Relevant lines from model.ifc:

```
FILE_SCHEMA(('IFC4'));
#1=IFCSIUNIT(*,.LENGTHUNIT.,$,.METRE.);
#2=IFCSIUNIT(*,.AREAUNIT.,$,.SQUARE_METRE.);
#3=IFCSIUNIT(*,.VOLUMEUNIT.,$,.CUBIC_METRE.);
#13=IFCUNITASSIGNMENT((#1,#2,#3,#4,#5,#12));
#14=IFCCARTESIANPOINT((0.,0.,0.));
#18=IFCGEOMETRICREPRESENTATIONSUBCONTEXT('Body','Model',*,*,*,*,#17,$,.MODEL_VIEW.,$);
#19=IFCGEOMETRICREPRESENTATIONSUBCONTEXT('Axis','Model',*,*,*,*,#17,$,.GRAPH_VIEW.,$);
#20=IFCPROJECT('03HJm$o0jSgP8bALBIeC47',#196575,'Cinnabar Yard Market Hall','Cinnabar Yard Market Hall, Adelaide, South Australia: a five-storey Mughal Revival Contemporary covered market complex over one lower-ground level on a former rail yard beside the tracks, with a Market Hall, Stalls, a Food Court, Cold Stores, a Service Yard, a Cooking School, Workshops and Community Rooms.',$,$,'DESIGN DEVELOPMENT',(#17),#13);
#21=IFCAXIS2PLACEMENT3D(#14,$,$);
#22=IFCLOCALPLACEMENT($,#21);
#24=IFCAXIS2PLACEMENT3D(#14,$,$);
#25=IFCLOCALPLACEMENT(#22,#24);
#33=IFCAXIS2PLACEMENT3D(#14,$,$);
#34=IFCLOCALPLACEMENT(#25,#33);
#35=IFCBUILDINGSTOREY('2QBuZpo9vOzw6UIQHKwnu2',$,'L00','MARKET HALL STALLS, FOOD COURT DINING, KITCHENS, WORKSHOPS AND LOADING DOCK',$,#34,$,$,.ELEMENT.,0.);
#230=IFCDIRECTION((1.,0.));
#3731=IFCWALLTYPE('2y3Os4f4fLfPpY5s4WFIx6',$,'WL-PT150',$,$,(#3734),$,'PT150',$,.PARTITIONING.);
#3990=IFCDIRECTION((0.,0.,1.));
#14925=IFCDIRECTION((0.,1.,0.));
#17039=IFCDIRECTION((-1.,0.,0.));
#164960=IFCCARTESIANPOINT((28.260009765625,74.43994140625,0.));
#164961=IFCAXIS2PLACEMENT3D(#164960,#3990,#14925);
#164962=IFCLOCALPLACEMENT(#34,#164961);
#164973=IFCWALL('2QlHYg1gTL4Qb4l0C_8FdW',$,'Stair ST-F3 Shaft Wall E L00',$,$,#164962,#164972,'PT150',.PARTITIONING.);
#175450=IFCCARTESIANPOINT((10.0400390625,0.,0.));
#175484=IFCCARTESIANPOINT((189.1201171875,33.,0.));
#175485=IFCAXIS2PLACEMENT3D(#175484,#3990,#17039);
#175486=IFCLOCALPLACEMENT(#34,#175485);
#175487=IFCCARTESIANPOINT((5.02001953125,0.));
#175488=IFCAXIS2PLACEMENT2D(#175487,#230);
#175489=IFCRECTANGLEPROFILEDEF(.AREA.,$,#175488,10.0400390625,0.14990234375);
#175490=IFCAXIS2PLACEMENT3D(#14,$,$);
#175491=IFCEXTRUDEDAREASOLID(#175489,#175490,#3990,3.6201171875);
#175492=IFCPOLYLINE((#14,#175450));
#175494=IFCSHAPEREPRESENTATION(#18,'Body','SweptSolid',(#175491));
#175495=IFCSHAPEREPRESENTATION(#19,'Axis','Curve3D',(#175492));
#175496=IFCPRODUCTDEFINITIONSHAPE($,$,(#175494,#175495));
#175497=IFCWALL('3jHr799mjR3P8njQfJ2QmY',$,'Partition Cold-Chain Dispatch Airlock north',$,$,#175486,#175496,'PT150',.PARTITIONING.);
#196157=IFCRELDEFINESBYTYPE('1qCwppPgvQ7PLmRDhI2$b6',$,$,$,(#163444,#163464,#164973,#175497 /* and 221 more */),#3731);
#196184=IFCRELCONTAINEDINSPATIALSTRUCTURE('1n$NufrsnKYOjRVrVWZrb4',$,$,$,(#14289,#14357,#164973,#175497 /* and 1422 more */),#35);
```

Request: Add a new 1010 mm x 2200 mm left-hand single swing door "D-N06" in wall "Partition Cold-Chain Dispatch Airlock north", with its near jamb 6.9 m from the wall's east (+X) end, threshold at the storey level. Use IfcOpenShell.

```python
import numpy as np
import ifcopenshell
import ifcopenshell.api.feature
import ifcopenshell.api.geometry
import ifcopenshell.api.root
import ifcopenshell.api.spatial
import ifcopenshell.geom
import ifcopenshell.util.element
import ifcopenshell.util.placement
import ifcopenshell.util.representation
import ifcopenshell.util.shape
import ifcopenshell.util.unit

model = ifcopenshell.open("model.ifc")
unit_scale = ifcopenshell.util.unit.calculate_unit_scale(model)
settings = ifcopenshell.geom.settings()


def volume(element):
    """Net volume in cubic metres, openings subtracted."""
    shape = ifcopenshell.geom.create_shape(settings, element)
    return ifcopenshell.util.shape.get_volume(shape.geometry)


wall = model.by_guid("3jHr799mjR3P8njQfJ2QmY")
storey = ifcopenshell.util.element.get_container(wall, ifc_class="IfcBuildingStorey")
context = ifcopenshell.util.representation.get_context(model, "Model", "Body", "MODEL_VIEW")
before = volume(wall)

width, height, from_end, sill = 1.01, 2.2, 6.9, 0.0  # metres

# The wall runs along its own X axis, and the end named is its -X end.
wall_shape = ifcopenshell.geom.create_shape(settings, wall)
x, y, z = ifcopenshell.util.shape.get_vertices(wall_shape.geometry).T
start = x.min() + from_end
face, thickness = float(y.min()), float(y.max() - y.min())
wall_matrix = ifcopenshell.util.placement.get_local_placement(wall.ObjectPlacement)
level = ifcopenshell.util.placement.get_local_placement(storey.ObjectPlacement)[2, 3]


def in_wall(x, y):
    """Placement at x, y metres in the wall's axes, at sill height."""
    matrix = wall_matrix.copy()
    matrix[:, 3] = wall_matrix @ np.array([x / unit_scale, y / unit_scale, 0.0, 1.0])
    matrix[2, 3] = level + sill / unit_scale
    return matrix


# Opening: a box that overshoots both wall faces by 50 mm.
opening = ifcopenshell.api.root.create_entity(model, ifc_class="IfcOpeningElement", predefined_type="OPENING")
box = ifcopenshell.api.geometry.add_wall_representation(
    model, context=context, length=width, height=height, thickness=thickness + 0.1
)
ifcopenshell.api.geometry.assign_representation(model, product=opening, representation=box)
ifcopenshell.api.geometry.edit_object_placement(model, product=opening, matrix=in_wall(start, face - 0.05), is_si=False)
ifcopenshell.api.feature.add_feature(model, feature=opening, element=wall)

door = ifcopenshell.api.root.create_entity(model, ifc_class="IfcDoor", name="D-N06", predefined_type="DOOR")
door.OverallWidth, door.OverallHeight = width / unit_scale, height / unit_scale
door.OperationType = "SINGLE_SWING_LEFT"
body = ifcopenshell.api.geometry.add_door_representation(
    model,
    context=context,
    overall_width=door.OverallWidth,
    overall_height=door.OverallHeight,
    operation_type="SINGLE_SWING_LEFT",
    lining_properties={"LiningDepth": thickness / unit_scale, "ThresholdDepth": thickness / unit_scale},
)
ifcopenshell.api.geometry.assign_representation(model, product=door, representation=body)
ifcopenshell.api.spatial.assign_container(model, products=[door], relating_structure=storey)
ifcopenshell.api.feature.add_filling(model, opening=opening, element=door)

# The lining spans the wall, so the door starts at the wall face.
ifcopenshell.api.geometry.edit_object_placement(model, product=door, matrix=in_wall(start, face), is_si=False)

after = volume(wall)

print(f"wall volume {before:.3f} -> {after:.3f} m3")

model.write("model_v2.ifc")
```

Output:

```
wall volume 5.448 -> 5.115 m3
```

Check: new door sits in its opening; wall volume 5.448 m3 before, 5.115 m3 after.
